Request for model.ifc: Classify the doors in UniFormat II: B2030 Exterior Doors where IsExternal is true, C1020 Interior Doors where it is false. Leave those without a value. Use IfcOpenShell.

First a look at what the model holds.

```python
import ifcopenshell
import ifcopenshell.util.element

model = ifcopenshell.open("model.ifc")
print(model.schema)
print("classifications:", [c.Name for c in model.by_type("IfcClassification")])
values = [ifcopenshell.util.element.get_pset(e, "Pset_DoorCommon", "IsExternal") for e in model.by_type("IfcDoor")]
for value in (True, False, None):
    print("IsExternal", value, values.count(value))
```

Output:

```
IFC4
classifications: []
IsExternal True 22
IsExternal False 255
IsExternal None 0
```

```python
import ifcopenshell
import ifcopenshell.api.classification
import ifcopenshell.util.element

model = ifcopenshell.open("model.ifc")

system = ifcopenshell.api.classification.add_classification(model, classification="UniFormat II")

doors = model.by_type("IfcDoor")
external = {e: ifcopenshell.util.element.get_pset(e, "Pset_DoorCommon", "IsExternal") for e in doors}
for flag, code, name in ((True, "B2030", "Exterior Doors"), (False, "C1020", "Interior Doors")):
    products = [e for e in doors if external[e] is flag]
    ifcopenshell.api.classification.add_reference(
        model, products=products, classification=system, identification=code, name=name
    )
    print(code, len(products))

model.write("model_v2.ifc")
```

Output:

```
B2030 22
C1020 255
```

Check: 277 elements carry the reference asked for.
